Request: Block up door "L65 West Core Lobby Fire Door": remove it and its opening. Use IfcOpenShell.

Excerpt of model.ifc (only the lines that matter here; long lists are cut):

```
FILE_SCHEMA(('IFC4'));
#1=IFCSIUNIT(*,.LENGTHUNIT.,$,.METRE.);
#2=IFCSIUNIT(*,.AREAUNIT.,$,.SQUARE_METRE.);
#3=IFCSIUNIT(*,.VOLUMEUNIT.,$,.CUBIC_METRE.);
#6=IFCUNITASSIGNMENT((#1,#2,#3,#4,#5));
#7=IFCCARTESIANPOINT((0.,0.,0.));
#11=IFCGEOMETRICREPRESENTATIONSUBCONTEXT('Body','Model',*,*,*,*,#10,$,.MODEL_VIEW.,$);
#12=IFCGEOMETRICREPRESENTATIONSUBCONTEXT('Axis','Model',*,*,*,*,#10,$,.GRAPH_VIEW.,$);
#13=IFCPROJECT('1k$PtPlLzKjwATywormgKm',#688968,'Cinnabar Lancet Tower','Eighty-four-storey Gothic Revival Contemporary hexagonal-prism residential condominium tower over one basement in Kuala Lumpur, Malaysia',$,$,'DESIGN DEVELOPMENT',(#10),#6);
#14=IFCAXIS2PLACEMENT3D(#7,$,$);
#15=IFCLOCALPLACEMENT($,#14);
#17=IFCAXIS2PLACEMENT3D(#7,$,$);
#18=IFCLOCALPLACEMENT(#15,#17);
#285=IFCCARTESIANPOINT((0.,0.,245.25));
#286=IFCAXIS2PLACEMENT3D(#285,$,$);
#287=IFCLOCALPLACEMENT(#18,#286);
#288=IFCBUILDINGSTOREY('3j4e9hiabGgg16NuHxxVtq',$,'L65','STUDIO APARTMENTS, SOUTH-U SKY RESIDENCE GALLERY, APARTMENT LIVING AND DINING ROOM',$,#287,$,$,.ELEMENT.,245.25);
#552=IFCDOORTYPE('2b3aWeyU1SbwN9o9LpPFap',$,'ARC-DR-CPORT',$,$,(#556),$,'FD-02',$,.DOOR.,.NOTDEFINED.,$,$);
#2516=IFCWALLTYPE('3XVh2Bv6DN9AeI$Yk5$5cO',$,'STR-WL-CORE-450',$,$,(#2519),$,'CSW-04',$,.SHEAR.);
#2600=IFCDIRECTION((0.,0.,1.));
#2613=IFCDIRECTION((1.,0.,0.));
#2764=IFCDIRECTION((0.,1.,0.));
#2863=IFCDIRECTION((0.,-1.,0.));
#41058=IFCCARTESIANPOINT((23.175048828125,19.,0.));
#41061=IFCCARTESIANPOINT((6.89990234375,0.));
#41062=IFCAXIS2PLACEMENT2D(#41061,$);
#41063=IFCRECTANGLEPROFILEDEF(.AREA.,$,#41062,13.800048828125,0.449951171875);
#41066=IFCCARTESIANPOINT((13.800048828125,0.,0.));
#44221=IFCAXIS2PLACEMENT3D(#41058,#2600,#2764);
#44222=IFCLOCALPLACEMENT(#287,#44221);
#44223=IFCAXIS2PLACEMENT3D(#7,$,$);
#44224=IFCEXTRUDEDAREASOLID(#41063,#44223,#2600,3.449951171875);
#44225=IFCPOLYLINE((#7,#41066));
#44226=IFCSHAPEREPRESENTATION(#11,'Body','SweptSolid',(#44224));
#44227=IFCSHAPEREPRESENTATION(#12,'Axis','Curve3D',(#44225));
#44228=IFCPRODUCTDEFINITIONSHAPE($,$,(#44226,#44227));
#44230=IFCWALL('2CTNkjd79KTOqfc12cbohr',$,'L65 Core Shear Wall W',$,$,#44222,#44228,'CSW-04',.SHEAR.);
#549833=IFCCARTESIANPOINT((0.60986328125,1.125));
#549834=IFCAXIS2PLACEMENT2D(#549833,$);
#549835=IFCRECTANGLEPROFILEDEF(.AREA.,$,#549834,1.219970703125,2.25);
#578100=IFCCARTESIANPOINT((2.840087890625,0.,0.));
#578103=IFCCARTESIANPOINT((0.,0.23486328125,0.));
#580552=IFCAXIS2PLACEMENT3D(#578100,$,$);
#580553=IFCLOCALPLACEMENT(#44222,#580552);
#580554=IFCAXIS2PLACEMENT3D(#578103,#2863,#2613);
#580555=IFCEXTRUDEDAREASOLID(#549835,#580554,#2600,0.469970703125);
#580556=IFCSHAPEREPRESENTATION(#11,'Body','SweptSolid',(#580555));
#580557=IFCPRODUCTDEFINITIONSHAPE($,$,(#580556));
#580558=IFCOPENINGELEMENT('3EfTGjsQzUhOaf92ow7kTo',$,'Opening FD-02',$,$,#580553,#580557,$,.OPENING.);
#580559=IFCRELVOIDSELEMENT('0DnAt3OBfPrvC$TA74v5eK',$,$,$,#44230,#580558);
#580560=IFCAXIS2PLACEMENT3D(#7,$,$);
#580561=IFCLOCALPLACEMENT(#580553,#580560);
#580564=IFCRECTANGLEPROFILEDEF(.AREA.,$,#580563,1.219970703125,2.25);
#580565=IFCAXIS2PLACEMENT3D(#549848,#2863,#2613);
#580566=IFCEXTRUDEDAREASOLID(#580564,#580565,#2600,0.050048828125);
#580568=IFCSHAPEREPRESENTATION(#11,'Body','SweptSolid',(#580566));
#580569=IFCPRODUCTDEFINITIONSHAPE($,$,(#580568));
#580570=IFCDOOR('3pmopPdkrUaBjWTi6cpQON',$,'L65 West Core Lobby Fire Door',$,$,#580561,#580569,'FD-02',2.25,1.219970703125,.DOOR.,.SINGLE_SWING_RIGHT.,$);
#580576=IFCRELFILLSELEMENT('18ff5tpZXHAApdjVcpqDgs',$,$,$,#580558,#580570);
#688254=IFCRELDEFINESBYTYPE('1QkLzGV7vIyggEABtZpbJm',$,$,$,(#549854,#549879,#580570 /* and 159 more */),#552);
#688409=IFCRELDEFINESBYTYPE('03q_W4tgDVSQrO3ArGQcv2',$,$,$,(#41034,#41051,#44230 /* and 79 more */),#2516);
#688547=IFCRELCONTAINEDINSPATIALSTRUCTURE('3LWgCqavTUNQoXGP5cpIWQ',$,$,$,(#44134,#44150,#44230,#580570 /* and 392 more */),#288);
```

```python
import ifcopenshell
import ifcopenshell.api.feature
import ifcopenshell.api.root
import ifcopenshell.geom
import ifcopenshell.util.shape

model = ifcopenshell.open("model.ifc")
settings = ifcopenshell.geom.settings()


def volume(element):
    """Net volume in cubic metres, openings subtracted."""
    shape = ifcopenshell.geom.create_shape(settings, element)
    return ifcopenshell.util.shape.get_volume(shape.geometry)


door = model.by_id(580570)
opening = door.FillsVoids[0].RelatingOpeningElement
wall = opening.VoidsElements[0].RelatingBuildingElement
before = volume(wall)

ifcopenshell.api.root.remove_product(model, product=door)
ifcopenshell.api.feature.remove_feature(model, feature=opening)

after = volume(wall)

print(f"wall volume {before:.3f} -> {after:.3f} m3")

model.write("model_edited.ifc")
```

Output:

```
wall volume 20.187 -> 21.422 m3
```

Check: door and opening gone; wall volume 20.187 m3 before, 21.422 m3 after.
